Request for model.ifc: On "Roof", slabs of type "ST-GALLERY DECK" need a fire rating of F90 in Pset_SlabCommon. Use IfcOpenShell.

First a look at what the model holds.

```python
import ifcopenshell
import ifcopenshell.util.element

model = ifcopenshell.open("model.ifc")
print(model.schema)
storey = next(s for s in model.by_type("IfcBuildingStorey") if s.Name == "Roof")
slabs = [e for e in ifcopenshell.util.element.get_decomposition(storey) if e.is_a("IfcSlab")]
seen = {}
for e in slabs:
    element_type = ifcopenshell.util.element.get_type(e)
    key = (element_type.Name if element_type != e and element_type else None, ifcopenshell.util.element.get_pset(e, "Pset_SlabCommon", "FireRating"))
    seen[key] = seen.get(key, 0) + 1
for (name, value), count in sorted(seen.items(), key=str):
    print(count, "x", name, "|", value)
```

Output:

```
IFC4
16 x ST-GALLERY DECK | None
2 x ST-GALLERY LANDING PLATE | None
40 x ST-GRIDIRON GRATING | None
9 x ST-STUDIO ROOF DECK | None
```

```python
import ifcopenshell
import ifcopenshell.api.pset
import ifcopenshell.util.element

model = ifcopenshell.open("model.ifc")

storey = next(s for s in model.by_type("IfcBuildingStorey") if s.Name == "Roof")
slabs = [e for e in ifcopenshell.util.element.get_decomposition(storey) if e.is_a("IfcSlab")]

count = 0
for e in slabs:
    element_type = ifcopenshell.util.element.get_type(e)
    if element_type in (None, e) or element_type.Name != "ST-GALLERY DECK":
        continue
    # add_pset returns the element's existing set when there is one.
    pset = ifcopenshell.api.pset.add_pset(model, product=e, name="Pset_SlabCommon")
    ifcopenshell.api.pset.edit_pset(model, pset=pset, properties={"FireRating": "F90"})
    count += 1

print(count, "slabs updated")

model.write("model_v2.ifc")
```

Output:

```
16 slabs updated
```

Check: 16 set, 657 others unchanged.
